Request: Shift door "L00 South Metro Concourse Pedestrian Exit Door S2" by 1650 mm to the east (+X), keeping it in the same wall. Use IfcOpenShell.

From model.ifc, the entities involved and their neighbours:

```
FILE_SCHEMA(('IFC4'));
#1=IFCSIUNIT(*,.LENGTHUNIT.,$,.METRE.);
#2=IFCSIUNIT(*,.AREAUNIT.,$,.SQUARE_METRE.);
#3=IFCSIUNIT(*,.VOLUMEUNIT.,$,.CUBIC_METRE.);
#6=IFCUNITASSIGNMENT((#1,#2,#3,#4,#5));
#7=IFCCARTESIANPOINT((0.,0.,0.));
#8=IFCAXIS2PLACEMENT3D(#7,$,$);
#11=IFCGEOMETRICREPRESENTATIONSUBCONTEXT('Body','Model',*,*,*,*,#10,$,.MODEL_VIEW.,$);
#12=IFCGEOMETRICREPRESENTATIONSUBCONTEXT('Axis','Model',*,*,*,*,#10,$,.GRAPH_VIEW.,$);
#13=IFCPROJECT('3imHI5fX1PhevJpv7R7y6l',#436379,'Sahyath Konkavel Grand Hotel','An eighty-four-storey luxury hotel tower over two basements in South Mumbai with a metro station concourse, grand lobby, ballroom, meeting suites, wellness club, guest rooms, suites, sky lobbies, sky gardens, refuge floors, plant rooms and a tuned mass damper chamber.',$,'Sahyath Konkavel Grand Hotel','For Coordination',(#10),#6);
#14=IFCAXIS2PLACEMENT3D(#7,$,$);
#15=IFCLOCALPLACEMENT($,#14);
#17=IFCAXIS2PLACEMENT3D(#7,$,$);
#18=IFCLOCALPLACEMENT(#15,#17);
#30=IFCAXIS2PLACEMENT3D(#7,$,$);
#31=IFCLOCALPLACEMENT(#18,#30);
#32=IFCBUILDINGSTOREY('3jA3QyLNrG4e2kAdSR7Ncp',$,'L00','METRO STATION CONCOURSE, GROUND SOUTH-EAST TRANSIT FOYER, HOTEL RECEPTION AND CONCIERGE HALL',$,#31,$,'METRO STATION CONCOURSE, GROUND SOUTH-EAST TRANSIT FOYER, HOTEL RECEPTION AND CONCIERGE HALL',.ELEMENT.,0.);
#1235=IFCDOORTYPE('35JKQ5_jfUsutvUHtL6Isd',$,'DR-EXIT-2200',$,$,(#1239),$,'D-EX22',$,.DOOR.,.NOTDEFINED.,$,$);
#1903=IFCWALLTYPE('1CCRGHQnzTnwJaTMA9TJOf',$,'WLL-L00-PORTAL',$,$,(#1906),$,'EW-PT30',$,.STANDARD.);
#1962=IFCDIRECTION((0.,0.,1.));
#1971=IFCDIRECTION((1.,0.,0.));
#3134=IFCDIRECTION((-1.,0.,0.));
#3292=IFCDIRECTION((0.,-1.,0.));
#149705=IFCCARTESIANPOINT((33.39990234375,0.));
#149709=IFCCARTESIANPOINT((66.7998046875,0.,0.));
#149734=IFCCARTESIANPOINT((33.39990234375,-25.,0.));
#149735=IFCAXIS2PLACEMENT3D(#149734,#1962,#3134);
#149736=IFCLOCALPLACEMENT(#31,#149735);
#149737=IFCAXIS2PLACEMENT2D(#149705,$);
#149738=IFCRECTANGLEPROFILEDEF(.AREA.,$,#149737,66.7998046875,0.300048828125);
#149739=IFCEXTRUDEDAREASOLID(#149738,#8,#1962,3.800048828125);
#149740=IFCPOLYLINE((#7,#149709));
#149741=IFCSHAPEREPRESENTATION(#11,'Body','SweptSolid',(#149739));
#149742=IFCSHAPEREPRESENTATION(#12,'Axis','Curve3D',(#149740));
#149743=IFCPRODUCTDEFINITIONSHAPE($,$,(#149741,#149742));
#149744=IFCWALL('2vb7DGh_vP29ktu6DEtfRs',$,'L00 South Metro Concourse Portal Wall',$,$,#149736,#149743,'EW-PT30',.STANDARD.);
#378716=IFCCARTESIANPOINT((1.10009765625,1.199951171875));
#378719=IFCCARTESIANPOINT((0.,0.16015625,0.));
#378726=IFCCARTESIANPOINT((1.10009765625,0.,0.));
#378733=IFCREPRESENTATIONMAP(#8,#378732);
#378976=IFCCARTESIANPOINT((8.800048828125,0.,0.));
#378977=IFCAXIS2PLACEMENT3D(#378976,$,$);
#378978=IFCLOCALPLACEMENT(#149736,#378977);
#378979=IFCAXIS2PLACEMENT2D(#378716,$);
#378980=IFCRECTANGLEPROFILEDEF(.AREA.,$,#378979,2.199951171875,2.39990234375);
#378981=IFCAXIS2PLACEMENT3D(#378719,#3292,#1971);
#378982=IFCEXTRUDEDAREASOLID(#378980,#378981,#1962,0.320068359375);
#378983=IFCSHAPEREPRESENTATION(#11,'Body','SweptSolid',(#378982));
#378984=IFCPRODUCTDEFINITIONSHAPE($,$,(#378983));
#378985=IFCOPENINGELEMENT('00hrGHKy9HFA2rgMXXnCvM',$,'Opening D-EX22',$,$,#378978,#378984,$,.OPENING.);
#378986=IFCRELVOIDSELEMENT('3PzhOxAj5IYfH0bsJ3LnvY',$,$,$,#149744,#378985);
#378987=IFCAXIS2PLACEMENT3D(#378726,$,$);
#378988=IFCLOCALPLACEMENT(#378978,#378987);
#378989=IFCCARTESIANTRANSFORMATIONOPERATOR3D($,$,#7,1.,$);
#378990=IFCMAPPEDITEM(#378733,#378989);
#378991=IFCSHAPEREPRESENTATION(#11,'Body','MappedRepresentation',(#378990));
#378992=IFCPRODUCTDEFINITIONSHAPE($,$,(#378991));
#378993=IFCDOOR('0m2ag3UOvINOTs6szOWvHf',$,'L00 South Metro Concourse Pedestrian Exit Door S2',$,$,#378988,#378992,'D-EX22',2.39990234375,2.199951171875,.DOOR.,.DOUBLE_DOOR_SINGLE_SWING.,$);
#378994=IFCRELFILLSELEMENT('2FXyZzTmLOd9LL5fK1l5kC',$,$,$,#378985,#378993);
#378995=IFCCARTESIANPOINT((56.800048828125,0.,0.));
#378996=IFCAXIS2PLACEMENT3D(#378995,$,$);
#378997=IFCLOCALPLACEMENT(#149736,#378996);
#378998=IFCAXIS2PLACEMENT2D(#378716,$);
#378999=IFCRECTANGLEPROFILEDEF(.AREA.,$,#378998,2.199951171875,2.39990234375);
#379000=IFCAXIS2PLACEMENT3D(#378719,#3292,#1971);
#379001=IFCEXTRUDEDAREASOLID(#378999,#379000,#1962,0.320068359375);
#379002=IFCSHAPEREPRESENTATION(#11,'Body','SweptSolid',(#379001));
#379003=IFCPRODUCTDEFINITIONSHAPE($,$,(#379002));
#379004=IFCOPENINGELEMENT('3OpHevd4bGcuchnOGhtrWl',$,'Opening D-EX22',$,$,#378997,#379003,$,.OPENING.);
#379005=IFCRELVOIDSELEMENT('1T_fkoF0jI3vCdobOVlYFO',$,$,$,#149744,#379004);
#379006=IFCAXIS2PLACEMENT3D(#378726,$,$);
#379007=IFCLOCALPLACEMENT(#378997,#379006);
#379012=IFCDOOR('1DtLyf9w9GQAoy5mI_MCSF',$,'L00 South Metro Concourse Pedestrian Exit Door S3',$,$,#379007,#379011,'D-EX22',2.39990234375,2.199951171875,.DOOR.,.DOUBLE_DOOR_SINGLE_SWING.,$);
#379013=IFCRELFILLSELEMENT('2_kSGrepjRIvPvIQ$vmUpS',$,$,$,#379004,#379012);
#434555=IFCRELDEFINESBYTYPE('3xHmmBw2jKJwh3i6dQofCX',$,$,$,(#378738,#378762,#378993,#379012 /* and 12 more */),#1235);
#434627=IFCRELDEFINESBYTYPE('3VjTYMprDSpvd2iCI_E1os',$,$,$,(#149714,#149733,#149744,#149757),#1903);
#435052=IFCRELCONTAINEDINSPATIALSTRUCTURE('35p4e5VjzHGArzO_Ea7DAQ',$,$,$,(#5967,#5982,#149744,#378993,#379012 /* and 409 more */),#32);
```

```python
import ifcopenshell
import ifcopenshell.api.geometry
import ifcopenshell.util.placement
import ifcopenshell.util.unit

model = ifcopenshell.open("model.ifc")
unit_scale = ifcopenshell.util.unit.calculate_unit_scale(model)

door = model.by_guid("0m2ag3UOvINOTs6szOWvHf")
opening = door.FillsVoids[0].RelatingOpeningElement
wall = opening.VoidsElements[0].RelatingBuildingElement

wall_matrix = ifcopenshell.util.placement.get_local_placement(wall.ObjectPlacement)
shift = wall_matrix[:3, 0] * -1.65 / unit_scale
before = ifcopenshell.util.placement.get_local_placement(door.ObjectPlacement)[:3, 3].copy()

# The door is placed relative to its opening, so it follows when the opening moves.
matrix = ifcopenshell.util.placement.get_local_placement(opening.ObjectPlacement)
matrix[:3, 3] += shift
ifcopenshell.api.geometry.edit_object_placement(
    model, product=opening, matrix=matrix, is_si=False, should_transform_children=True
)

after = ifcopenshell.util.placement.get_local_placement(door.ObjectPlacement)[:3, 3]
print("door moved by", (after - before).round(3) + 0.0)

model.write("model_edited.ifc")
```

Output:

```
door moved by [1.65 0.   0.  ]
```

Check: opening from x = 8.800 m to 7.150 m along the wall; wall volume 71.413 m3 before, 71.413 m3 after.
